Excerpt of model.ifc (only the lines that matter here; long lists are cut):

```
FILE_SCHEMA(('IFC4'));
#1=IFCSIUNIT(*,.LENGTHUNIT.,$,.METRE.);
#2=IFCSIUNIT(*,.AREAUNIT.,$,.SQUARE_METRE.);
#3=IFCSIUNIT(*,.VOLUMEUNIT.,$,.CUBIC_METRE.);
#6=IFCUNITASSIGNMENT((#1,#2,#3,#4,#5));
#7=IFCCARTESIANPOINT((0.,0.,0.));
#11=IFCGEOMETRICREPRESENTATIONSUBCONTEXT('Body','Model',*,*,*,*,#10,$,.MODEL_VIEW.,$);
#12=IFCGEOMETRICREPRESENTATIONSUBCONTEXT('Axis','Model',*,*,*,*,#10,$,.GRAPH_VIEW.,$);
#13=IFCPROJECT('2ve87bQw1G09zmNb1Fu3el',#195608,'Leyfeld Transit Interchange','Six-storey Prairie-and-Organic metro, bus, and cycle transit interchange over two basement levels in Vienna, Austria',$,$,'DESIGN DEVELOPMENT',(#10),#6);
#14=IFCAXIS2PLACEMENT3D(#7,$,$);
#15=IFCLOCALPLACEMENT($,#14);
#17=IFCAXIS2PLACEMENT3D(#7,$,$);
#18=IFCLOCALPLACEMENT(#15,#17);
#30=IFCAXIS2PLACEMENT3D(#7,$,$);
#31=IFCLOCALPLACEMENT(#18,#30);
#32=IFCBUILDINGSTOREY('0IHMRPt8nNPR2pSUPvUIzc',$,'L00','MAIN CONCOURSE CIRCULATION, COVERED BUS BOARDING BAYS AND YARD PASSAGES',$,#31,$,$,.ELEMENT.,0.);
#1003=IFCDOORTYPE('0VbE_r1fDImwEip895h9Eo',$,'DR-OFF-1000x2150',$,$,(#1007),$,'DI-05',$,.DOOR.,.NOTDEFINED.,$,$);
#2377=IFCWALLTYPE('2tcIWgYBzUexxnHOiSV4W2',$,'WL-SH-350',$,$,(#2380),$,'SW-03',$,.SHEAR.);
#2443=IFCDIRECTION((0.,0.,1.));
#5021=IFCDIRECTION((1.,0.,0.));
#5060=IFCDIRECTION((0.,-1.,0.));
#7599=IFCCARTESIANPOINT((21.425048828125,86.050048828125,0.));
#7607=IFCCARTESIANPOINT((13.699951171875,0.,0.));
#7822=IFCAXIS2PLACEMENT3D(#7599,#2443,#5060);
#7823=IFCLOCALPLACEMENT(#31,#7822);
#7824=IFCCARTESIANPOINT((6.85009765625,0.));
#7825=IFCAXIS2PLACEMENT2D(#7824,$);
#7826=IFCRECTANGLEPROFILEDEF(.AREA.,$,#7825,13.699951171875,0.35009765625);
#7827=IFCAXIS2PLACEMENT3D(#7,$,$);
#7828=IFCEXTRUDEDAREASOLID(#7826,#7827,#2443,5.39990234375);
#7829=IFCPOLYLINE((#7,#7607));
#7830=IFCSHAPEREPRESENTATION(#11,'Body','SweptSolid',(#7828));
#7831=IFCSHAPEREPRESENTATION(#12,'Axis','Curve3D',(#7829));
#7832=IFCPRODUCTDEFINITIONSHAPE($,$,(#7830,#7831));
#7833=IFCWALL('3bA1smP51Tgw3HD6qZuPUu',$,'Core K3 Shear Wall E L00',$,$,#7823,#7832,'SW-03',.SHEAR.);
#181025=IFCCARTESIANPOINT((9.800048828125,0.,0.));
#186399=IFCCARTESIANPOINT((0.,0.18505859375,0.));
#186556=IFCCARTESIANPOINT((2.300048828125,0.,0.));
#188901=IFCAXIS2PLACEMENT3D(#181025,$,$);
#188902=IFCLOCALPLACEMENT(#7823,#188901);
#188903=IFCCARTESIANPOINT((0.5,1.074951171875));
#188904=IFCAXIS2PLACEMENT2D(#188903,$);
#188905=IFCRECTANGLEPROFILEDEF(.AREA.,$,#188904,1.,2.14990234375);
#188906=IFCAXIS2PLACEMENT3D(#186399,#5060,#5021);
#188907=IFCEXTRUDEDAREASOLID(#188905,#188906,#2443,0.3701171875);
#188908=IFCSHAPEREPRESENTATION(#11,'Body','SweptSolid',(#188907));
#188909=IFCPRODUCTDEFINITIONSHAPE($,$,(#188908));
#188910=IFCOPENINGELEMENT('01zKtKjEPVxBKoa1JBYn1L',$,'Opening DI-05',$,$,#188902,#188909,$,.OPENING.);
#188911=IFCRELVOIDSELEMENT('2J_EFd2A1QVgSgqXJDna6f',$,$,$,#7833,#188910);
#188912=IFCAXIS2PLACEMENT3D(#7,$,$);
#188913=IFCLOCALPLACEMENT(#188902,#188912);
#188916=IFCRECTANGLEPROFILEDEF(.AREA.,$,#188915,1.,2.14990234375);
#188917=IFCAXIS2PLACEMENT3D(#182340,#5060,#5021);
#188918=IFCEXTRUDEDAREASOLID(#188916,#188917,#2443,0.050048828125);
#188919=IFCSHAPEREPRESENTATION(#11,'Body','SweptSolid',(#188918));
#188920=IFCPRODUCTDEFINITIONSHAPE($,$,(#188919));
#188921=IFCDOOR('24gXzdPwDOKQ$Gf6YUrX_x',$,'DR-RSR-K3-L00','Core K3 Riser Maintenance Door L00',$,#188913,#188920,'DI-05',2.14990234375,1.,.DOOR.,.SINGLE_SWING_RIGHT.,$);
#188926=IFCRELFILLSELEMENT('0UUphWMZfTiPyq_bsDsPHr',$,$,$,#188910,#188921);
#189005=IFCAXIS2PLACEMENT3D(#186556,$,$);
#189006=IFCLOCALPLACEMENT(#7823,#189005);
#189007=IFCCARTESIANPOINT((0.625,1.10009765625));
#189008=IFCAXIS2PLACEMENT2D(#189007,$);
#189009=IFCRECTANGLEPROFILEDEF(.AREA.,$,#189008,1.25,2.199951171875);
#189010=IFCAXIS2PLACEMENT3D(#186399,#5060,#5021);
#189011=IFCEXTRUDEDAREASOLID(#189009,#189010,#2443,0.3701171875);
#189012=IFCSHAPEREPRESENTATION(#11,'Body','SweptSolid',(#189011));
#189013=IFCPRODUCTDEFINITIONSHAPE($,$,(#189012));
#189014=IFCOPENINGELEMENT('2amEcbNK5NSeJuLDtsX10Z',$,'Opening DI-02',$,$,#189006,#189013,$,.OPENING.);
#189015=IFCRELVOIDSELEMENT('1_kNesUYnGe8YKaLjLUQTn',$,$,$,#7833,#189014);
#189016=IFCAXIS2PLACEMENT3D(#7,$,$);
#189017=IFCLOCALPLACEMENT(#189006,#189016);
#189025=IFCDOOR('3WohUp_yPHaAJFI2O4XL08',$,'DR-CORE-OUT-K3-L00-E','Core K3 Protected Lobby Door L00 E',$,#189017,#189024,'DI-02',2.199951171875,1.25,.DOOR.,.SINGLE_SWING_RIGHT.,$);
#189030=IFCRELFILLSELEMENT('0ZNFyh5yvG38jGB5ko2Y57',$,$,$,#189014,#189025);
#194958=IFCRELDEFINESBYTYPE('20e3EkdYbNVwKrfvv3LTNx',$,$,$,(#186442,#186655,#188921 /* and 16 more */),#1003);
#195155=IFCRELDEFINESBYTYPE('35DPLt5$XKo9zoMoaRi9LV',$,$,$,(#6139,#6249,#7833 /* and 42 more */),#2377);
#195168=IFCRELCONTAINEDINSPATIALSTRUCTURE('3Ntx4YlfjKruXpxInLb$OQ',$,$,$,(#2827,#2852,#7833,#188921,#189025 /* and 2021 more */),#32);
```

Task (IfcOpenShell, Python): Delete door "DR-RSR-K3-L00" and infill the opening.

```python
import ifcopenshell
import ifcopenshell.api.feature
import ifcopenshell.api.root
import ifcopenshell.geom
import ifcopenshell.util.shape

model = ifcopenshell.open("model.ifc")
settings = ifcopenshell.geom.settings()


def volume(element):
    """Net volume in cubic metres, openings subtracted."""
    shape = ifcopenshell.geom.create_shape(settings, element)
    return ifcopenshell.util.shape.get_volume(shape.geometry)


door = model.by_guid("24gXzdPwDOKQ$Gf6YUrX_x")
opening = door.FillsVoids[0].RelatingOpeningElement
wall = opening.VoidsElements[0].RelatingBuildingElement
before = volume(wall)

ifcopenshell.api.root.remove_product(model, product=door)
ifcopenshell.api.feature.remove_feature(model, feature=opening)

after = volume(wall)

print(f"wall volume {before:.3f} -> {after:.3f} m3")

model.write("model_edited.ifc")
```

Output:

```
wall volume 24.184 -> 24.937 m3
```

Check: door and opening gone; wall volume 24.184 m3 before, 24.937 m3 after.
